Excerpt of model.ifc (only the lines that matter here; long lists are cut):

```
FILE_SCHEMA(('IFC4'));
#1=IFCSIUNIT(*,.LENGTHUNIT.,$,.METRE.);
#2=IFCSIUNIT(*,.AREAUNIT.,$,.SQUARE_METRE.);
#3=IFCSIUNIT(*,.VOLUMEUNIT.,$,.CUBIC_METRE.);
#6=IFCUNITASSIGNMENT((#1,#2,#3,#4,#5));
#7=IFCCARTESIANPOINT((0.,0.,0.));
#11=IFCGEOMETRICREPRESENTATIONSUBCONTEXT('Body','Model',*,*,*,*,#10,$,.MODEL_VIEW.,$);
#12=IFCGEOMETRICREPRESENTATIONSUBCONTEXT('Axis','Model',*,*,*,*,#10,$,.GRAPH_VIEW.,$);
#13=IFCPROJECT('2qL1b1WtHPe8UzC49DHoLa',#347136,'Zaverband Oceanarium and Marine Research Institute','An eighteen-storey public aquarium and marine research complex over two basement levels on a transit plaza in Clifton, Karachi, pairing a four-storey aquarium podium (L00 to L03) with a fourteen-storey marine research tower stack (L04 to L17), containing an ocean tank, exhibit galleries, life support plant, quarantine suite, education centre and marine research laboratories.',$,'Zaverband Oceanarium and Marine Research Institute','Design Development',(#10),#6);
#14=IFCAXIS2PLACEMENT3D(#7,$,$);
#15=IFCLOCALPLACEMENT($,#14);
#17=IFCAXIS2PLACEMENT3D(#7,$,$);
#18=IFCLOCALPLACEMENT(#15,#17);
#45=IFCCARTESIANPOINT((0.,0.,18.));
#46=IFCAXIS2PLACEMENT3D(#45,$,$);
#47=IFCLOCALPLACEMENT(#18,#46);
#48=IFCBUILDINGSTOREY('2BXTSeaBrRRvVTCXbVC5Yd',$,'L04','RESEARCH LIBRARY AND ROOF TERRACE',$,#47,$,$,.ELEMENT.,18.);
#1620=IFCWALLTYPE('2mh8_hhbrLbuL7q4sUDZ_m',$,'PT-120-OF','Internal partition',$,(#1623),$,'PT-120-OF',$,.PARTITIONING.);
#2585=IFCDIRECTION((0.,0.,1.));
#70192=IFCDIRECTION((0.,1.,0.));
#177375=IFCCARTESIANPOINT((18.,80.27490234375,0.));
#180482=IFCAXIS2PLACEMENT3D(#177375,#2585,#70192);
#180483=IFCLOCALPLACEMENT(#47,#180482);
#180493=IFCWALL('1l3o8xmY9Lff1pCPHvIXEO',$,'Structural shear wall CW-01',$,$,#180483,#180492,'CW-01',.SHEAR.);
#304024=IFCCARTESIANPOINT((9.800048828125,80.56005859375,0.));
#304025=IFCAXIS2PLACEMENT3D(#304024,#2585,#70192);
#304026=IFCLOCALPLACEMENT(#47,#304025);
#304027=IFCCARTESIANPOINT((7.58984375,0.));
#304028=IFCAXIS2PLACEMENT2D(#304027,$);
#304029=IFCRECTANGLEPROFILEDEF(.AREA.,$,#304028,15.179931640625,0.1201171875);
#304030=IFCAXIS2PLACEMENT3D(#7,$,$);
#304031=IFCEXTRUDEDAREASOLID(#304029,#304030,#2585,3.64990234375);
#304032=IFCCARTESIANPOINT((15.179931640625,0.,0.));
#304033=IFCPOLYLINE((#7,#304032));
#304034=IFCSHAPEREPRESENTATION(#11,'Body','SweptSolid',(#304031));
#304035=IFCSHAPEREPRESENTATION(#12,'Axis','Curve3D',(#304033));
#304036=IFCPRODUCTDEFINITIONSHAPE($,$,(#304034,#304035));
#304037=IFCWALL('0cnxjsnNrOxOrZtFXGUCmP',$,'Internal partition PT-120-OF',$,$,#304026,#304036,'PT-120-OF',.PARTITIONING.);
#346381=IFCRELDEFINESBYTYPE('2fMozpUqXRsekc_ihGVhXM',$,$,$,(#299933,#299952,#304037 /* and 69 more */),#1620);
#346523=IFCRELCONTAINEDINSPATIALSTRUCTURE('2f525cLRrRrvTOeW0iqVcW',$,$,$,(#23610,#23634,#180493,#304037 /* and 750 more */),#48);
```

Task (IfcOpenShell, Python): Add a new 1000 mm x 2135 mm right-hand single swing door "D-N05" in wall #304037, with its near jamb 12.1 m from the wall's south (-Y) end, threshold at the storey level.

```python
import numpy as np
import ifcopenshell
import ifcopenshell.api.feature
import ifcopenshell.api.geometry
import ifcopenshell.api.root
import ifcopenshell.api.spatial
import ifcopenshell.geom
import ifcopenshell.util.element
import ifcopenshell.util.placement
import ifcopenshell.util.representation
import ifcopenshell.util.shape
import ifcopenshell.util.unit

model = ifcopenshell.open("model.ifc")
unit_scale = ifcopenshell.util.unit.calculate_unit_scale(model)
settings = ifcopenshell.geom.settings()


def volume(element):
    """Net volume in cubic metres, openings subtracted."""
    shape = ifcopenshell.geom.create_shape(settings, element)
    return ifcopenshell.util.shape.get_volume(shape.geometry)


wall = model.by_guid("0cnxjsnNrOxOrZtFXGUCmP")
storey = ifcopenshell.util.element.get_container(wall, ifc_class="IfcBuildingStorey")
context = ifcopenshell.util.representation.get_context(model, "Model", "Body", "MODEL_VIEW")
before = volume(wall)

width, height, from_end, sill = 1, 2.135, 12.1, 0.0  # metres

# The wall runs along its own X axis, and the end named is its -X end.
wall_shape = ifcopenshell.geom.create_shape(settings, wall)
x, y, z = ifcopenshell.util.shape.get_vertices(wall_shape.geometry).T
start = x.min() + from_end
face, thickness = float(y.min()), float(y.max() - y.min())
wall_matrix = ifcopenshell.util.placement.get_local_placement(wall.ObjectPlacement)
level = ifcopenshell.util.placement.get_local_placement(storey.ObjectPlacement)[2, 3]


def in_wall(x, y):
    """Placement at x, y metres in the wall's axes, at sill height."""
    matrix = wall_matrix.copy()
    matrix[:, 3] = wall_matrix @ np.array([x / unit_scale, y / unit_scale, 0.0, 1.0])
    matrix[2, 3] = level + sill / unit_scale
    return matrix


# Opening: a box that overshoots both wall faces by 50 mm.
opening = ifcopenshell.api.root.create_entity(model, ifc_class="IfcOpeningElement", predefined_type="OPENING")
box = ifcopenshell.api.geometry.add_wall_representation(
    model, context=context, length=width, height=height, thickness=thickness + 0.1
)
ifcopenshell.api.geometry.assign_representation(model, product=opening, representation=box)
ifcopenshell.api.geometry.edit_object_placement(model, product=opening, matrix=in_wall(start, face - 0.05), is_si=False)
ifcopenshell.api.feature.add_feature(model, feature=opening, element=wall)

door = ifcopenshell.api.root.create_entity(model, ifc_class="IfcDoor", name="D-N05", predefined_type="DOOR")
door.OverallWidth, door.OverallHeight = width / unit_scale, height / unit_scale
door.OperationType = "SINGLE_SWING_RIGHT"
body = ifcopenshell.api.geometry.add_door_representation(
    model,
    context=context,
    overall_width=door.OverallWidth,
    overall_height=door.OverallHeight,
    operation_type="SINGLE_SWING_RIGHT",
    lining_properties={"LiningDepth": thickness / unit_scale, "ThresholdDepth": thickness / unit_scale},
)
ifcopenshell.api.geometry.assign_representation(model, product=door, representation=body)
ifcopenshell.api.spatial.assign_container(model, products=[door], relating_structure=storey)
ifcopenshell.api.feature.add_filling(model, opening=opening, element=door)

# The lining spans the wall, so the door starts at the wall face.
ifcopenshell.api.geometry.edit_object_placement(model, product=door, matrix=in_wall(start, face), is_si=False)

after = volume(wall)

print(f"wall volume {before:.3f} -> {after:.3f} m3")

model.write("model-out.ifc")
```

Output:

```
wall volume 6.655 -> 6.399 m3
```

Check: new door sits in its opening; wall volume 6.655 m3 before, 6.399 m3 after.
